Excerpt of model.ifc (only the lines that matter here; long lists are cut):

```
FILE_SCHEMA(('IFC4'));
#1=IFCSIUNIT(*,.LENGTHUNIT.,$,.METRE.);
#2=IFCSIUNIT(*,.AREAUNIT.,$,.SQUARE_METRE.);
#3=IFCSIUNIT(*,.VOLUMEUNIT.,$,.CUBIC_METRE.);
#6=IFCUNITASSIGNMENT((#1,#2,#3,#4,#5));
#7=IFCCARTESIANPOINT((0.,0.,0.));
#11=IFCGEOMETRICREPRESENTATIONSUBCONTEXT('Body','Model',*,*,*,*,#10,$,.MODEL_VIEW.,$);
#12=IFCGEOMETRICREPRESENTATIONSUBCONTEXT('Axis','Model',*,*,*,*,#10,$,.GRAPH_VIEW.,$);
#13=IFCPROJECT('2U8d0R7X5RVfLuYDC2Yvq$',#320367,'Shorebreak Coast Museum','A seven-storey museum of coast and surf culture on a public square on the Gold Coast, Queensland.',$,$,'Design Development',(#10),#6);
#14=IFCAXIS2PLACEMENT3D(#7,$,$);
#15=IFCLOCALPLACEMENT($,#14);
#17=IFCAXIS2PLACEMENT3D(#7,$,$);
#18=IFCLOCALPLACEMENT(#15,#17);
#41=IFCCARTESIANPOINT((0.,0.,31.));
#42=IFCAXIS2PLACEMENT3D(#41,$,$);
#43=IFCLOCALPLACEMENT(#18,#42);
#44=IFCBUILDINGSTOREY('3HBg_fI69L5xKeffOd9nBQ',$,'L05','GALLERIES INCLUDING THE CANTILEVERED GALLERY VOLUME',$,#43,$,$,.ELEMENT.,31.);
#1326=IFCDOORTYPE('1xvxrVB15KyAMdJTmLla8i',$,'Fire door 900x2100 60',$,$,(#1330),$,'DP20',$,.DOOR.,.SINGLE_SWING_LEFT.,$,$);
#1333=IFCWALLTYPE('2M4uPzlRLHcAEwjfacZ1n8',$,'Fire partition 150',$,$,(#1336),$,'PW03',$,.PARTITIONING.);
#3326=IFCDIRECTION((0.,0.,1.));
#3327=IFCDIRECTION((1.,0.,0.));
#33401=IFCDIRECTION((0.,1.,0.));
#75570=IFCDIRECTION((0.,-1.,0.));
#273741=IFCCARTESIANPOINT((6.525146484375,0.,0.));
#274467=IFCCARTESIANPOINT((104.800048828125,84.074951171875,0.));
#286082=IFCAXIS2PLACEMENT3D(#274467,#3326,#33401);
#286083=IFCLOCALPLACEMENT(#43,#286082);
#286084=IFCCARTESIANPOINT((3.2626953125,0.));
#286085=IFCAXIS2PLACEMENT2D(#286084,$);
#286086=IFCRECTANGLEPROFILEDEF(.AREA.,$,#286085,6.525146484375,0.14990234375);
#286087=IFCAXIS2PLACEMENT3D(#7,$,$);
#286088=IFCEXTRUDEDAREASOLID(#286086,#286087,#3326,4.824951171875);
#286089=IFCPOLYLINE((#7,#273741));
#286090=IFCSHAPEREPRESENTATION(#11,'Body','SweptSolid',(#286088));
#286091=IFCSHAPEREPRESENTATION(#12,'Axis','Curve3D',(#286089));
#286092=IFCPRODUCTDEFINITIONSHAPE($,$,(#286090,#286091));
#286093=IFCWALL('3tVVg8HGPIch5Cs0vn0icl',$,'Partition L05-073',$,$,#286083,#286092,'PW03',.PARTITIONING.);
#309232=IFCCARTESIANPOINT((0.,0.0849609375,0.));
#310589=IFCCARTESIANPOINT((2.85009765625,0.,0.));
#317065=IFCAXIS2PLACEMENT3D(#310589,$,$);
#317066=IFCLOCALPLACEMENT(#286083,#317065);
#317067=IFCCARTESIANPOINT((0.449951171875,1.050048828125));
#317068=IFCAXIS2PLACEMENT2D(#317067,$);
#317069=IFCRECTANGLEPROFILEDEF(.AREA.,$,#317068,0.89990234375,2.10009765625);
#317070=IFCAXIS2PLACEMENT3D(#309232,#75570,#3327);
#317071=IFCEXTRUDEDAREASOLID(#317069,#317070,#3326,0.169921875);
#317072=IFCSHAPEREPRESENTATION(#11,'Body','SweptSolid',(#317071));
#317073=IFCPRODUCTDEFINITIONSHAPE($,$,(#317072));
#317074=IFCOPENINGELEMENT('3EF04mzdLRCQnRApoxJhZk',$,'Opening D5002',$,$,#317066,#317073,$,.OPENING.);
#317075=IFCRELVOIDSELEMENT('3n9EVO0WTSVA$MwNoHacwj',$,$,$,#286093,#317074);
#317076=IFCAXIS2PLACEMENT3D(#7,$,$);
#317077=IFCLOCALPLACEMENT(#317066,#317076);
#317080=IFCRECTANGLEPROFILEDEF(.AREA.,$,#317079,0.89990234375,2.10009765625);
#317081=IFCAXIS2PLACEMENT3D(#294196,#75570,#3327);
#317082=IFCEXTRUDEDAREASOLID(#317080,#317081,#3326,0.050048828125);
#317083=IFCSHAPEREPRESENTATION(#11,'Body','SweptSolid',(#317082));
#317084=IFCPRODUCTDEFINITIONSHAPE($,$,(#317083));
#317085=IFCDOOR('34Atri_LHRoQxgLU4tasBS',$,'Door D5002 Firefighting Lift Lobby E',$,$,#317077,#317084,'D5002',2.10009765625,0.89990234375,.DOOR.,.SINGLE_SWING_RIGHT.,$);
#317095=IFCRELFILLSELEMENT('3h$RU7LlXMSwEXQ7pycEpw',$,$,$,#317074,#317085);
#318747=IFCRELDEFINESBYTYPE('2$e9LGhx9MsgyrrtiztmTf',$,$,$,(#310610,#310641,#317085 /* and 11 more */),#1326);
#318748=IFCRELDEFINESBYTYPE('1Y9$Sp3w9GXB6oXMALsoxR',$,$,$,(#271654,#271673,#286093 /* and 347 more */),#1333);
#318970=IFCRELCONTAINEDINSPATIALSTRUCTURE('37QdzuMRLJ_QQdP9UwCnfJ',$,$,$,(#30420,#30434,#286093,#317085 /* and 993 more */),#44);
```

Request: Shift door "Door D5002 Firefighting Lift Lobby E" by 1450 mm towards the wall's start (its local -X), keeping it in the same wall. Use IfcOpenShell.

```python
import ifcopenshell
import ifcopenshell.api.geometry
import ifcopenshell.util.placement
import ifcopenshell.util.unit

model = ifcopenshell.open("model.ifc")
unit_scale = ifcopenshell.util.unit.calculate_unit_scale(model)

door = model.by_guid("34Atri_LHRoQxgLU4tasBS")
opening = door.FillsVoids[0].RelatingOpeningElement
wall = opening.VoidsElements[0].RelatingBuildingElement

wall_matrix = ifcopenshell.util.placement.get_local_placement(wall.ObjectPlacement)
shift = wall_matrix[:3, 0] * -1.45 / unit_scale
before = ifcopenshell.util.placement.get_local_placement(door.ObjectPlacement)[:3, 3].copy()

# The door is placed relative to its opening, so it follows when the opening moves.
matrix = ifcopenshell.util.placement.get_local_placement(opening.ObjectPlacement)
matrix[:3, 3] += shift
ifcopenshell.api.geometry.edit_object_placement(
    model, product=opening, matrix=matrix, is_si=False, should_transform_children=True
)

after = ifcopenshell.util.placement.get_local_placement(door.ObjectPlacement)[:3, 3]
print("door moved by", (after - before).round(3) + 0.0)

model.write("model_edited.ifc")
```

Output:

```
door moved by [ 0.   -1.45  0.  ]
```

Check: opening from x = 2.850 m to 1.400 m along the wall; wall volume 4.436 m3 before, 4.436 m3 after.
